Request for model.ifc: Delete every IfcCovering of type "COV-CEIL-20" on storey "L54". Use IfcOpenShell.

First a look at what the model holds.

```python
import ifcopenshell
import ifcopenshell.util.element

model = ifcopenshell.open("model.ifc")
print(model.schema)
storey = next(s for s in model.by_type("IfcBuildingStorey") if s.Name == "L54")
coverings = [e for e in ifcopenshell.util.element.get_decomposition(storey) if e.is_a("IfcCovering")]
seen = {}
for e in coverings:
    element_type = ifcopenshell.util.element.get_type(e)
    name = element_type.Name if element_type not in (None, e) else None
    seen[name] = seen.get(name, 0) + 1
for name, count in sorted(seen.items(), key=str):
    print(count, "x", name)
```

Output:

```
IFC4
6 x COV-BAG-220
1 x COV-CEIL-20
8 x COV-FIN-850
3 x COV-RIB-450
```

```python
import ifcopenshell
import ifcopenshell.api.root
import ifcopenshell.util.element

model = ifcopenshell.open("model.ifc")

storey = next(s for s in model.by_type("IfcBuildingStorey") if s.Name == "L54")
coverings = [e for e in ifcopenshell.util.element.get_decomposition(storey) if e.is_a("IfcCovering")]
targets = [e for e in coverings if (t := ifcopenshell.util.element.get_type(e)) not in (None, e) and t.Name == "COV-CEIL-20"]

for e in targets:
    ifcopenshell.api.root.remove_product(model, product=e)
print(len(targets), "removed")

model.write("model_rev.ifc")
```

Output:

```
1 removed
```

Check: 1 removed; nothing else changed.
